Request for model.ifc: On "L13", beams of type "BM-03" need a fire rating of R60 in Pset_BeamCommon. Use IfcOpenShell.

First a look at what the model holds.

```python
import ifcopenshell
import ifcopenshell.util.element

model = ifcopenshell.open("model.ifc")
print(model.schema)
storey = next(s for s in model.by_type("IfcBuildingStorey") if s.Name == "L13")
beams = [e for e in ifcopenshell.util.element.get_decomposition(storey) if e.is_a("IfcBeam")]
seen = {}
for e in beams:
    element_type = ifcopenshell.util.element.get_type(e)
    key = (element_type.Name if element_type != e and element_type else None, ifcopenshell.util.element.get_pset(e, "Pset_BeamCommon", "FireRating"))
    seen[key] = seen.get(key, 0) + 1
for (name, value), count in sorted(seen.items(), key=str):
    print(count, "x", name, "|", value)
```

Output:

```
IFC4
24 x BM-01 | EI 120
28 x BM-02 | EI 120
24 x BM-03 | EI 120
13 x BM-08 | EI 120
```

```python
import ifcopenshell
import ifcopenshell.api.pset
import ifcopenshell.util.element

model = ifcopenshell.open("model.ifc")

storey = next(s for s in model.by_type("IfcBuildingStorey") if s.Name == "L13")
beams = [e for e in ifcopenshell.util.element.get_decomposition(storey) if e.is_a("IfcBeam")]

count = 0
for e in beams:
    element_type = ifcopenshell.util.element.get_type(e)
    if element_type in (None, e) or element_type.Name != "BM-03":
        continue
    # add_pset returns the element's existing set when there is one.
    pset = ifcopenshell.api.pset.add_pset(model, product=e, name="Pset_BeamCommon")
    ifcopenshell.api.pset.edit_pset(model, pset=pset, properties={"FireRating": "R60"})
    count += 1

print(count, "beams updated")

model.write("model_updated.ifc")
```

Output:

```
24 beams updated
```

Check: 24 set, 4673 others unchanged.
